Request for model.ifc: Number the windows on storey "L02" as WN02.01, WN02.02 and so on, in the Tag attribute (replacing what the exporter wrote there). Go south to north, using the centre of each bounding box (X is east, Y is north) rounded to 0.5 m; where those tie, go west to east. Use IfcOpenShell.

First a look at what the model holds.

```python
import ifcopenshell
import ifcopenshell.util.element
import ifcopenshell.util.placement

model = ifcopenshell.open("model.ifc")
print(model.schema)
storey = next(s for s in model.by_type("IfcBuildingStorey") if s.Name == "L02")
windows = [e for e in ifcopenshell.util.element.get_decomposition(storey) if e.is_a("IfcWindow")]
for e in sorted(windows, key=lambda e: e.id()):
    origin = ifcopenshell.util.placement.get_local_placement(e.ObjectPlacement)[:3, 3]
    print(e.id(), e.Tag, e.Name, origin.round(2) + 0.0, sep=" | ")
```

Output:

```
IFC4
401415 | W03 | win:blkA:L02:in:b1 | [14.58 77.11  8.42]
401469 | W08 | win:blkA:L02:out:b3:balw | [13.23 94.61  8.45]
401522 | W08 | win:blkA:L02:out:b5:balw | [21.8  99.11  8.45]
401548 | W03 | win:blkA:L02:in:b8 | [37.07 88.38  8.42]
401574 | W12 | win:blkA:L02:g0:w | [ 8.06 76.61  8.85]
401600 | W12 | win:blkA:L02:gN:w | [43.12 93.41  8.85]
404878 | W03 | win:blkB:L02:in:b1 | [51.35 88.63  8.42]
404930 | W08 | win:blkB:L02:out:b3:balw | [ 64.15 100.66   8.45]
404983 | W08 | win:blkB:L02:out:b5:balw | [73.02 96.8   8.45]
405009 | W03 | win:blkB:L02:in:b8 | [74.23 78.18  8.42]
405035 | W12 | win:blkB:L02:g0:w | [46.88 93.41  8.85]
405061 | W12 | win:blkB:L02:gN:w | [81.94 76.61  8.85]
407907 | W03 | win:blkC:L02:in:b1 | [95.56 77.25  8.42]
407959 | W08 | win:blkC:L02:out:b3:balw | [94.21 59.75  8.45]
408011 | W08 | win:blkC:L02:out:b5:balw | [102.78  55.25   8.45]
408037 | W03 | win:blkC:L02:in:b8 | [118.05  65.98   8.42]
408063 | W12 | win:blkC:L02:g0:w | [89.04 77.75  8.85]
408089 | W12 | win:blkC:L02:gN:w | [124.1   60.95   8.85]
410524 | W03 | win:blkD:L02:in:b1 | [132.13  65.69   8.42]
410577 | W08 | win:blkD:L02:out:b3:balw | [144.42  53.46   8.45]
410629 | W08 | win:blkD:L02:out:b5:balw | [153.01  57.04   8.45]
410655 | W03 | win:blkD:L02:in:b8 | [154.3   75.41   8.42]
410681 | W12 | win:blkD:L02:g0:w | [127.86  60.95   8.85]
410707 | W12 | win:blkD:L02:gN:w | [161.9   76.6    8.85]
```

```python
import ifcopenshell
import ifcopenshell.geom
import ifcopenshell.util.element
import ifcopenshell.util.shape

model = ifcopenshell.open("model.ifc")
settings = ifcopenshell.geom.settings()
settings.set("use-world-coords", True)


def centre(element):
    shape = ifcopenshell.geom.create_shape(settings, element)
    return ifcopenshell.util.shape.get_bbox_centroid(shape.geometry)


storey = next(s for s in model.by_type("IfcBuildingStorey") if s.Name == "L02")
windows = [e for e in ifcopenshell.util.element.get_decomposition(storey) if e.is_a("IfcWindow")]

# Insertion points can sit at a corner or the storey origin, so sort by the geometry (in metres).
centres = {e: centre(e) for e in windows}
windows.sort(key=lambda e: (round(centres[e][1] / 0.5), centres[e][0]))

for i, e in enumerate(windows, start=1):
    number = f"WN02.{i:02d}"
    e.Tag = number
    print(e.id(), number)

model.write("model_updated.ifc")
```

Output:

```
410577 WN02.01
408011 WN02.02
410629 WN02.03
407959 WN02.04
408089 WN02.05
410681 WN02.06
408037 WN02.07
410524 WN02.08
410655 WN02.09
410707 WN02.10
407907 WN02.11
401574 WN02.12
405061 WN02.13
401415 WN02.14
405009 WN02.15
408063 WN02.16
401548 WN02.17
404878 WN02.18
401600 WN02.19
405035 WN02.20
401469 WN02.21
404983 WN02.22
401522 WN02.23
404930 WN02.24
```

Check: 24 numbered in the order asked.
